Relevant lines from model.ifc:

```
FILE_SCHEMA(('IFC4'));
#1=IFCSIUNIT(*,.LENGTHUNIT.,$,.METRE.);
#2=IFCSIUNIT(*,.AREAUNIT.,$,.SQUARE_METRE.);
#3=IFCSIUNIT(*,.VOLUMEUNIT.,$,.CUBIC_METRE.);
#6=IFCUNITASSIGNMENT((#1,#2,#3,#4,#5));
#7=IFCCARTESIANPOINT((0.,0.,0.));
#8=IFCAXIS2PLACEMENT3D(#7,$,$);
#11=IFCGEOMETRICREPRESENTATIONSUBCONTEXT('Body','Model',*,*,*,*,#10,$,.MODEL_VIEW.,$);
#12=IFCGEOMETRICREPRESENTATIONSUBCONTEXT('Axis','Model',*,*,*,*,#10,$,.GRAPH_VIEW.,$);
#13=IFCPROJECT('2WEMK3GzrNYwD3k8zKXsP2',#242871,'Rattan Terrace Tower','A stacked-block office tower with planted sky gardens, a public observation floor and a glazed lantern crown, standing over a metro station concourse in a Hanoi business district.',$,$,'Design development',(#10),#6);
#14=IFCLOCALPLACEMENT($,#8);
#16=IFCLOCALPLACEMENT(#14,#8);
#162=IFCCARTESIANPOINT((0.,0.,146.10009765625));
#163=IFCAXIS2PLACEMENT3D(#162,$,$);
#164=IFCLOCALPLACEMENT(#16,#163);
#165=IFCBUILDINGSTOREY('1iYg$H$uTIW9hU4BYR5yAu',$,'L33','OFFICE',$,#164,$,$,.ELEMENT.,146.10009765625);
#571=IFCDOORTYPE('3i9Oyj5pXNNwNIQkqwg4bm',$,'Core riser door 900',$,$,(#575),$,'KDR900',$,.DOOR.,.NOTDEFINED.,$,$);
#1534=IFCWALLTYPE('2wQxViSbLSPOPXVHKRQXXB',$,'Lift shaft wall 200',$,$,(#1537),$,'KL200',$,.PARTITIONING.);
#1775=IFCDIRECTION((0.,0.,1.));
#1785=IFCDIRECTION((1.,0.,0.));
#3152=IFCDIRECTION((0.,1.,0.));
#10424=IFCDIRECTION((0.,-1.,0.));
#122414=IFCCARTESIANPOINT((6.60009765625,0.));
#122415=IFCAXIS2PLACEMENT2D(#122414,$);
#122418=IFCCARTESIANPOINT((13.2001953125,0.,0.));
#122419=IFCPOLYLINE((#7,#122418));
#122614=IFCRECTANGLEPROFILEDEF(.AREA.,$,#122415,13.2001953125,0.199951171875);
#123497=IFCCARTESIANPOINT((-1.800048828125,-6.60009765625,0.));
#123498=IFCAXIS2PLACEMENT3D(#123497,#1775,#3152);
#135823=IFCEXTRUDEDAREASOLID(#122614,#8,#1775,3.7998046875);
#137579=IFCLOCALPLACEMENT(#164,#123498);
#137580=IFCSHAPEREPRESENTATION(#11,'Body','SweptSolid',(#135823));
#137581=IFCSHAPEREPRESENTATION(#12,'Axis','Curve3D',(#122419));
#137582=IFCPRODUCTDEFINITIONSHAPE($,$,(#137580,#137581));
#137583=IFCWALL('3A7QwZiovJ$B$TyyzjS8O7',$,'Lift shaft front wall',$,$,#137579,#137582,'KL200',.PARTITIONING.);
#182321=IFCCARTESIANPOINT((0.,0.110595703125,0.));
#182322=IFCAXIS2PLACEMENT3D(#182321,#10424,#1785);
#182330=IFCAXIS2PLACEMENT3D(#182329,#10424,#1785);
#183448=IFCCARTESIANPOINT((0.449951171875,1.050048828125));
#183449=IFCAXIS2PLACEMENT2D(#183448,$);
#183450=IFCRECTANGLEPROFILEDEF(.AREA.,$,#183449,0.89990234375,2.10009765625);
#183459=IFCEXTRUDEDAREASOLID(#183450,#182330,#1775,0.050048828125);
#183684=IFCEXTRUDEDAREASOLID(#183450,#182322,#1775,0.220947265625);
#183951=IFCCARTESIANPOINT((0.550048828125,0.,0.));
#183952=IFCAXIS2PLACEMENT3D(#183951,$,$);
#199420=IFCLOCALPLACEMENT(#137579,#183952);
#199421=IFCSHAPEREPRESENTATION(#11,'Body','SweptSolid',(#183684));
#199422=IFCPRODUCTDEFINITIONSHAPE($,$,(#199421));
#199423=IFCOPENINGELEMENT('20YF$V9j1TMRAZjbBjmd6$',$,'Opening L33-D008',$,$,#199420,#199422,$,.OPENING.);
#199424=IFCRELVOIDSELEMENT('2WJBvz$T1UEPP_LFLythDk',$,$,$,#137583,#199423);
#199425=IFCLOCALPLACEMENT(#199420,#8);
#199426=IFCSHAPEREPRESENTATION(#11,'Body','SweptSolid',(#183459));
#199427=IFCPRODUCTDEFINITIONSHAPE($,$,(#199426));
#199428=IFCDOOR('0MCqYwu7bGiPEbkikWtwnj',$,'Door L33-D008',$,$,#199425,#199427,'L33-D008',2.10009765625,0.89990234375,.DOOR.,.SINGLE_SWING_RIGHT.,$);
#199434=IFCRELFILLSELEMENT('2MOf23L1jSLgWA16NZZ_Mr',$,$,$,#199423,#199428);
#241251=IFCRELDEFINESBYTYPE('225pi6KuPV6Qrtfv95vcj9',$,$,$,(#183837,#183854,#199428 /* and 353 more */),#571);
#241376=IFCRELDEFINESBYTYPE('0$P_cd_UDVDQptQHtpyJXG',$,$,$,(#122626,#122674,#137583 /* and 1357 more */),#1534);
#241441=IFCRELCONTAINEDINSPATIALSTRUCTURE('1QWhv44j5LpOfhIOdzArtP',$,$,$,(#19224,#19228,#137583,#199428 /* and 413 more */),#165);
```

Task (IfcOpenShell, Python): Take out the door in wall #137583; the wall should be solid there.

```python
import ifcopenshell
import ifcopenshell.api.feature
import ifcopenshell.api.root
import ifcopenshell.geom
import ifcopenshell.util.shape

model = ifcopenshell.open("model.ifc")
settings = ifcopenshell.geom.settings()


def volume(element):
    """Net volume in cubic metres, openings subtracted."""
    shape = ifcopenshell.geom.create_shape(settings, element)
    return ifcopenshell.util.shape.get_volume(shape.geometry)


door = model.by_guid("0MCqYwu7bGiPEbkikWtwnj")
opening = door.FillsVoids[0].RelatingOpeningElement
wall = opening.VoidsElements[0].RelatingBuildingElement
before = volume(wall)

ifcopenshell.api.root.remove_product(model, product=door)
ifcopenshell.api.feature.remove_feature(model, feature=opening)

after = volume(wall)

print(f"wall volume {before:.3f} -> {after:.3f} m3")

model.write("model-out.ifc")
```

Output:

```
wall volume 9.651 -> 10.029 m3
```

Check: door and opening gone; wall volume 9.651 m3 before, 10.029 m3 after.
